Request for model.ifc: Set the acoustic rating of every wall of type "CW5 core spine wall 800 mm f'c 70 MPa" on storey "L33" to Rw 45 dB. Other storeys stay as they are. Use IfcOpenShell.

First a look at what the model holds.

```python
import ifcopenshell
import ifcopenshell.util.element

model = ifcopenshell.open("model.ifc")
print(model.schema)
storey = next(s for s in model.by_type("IfcBuildingStorey") if s.Name == "L33")
walls = [e for e in ifcopenshell.util.element.get_decomposition(storey) if e.is_a("IfcWall")]
seen = {}
for e in walls:
    element_type = ifcopenshell.util.element.get_type(e)
    key = (element_type.Name if element_type != e and element_type else None, ifcopenshell.util.element.get_pset(e, "Pset_WallCommon", "AcousticRating"))
    seen[key] = seen.get(key, 0) + 1
for (name, value), count in sorted(seen.items(), key=str):
    print(count, "x", name, "|", value)
```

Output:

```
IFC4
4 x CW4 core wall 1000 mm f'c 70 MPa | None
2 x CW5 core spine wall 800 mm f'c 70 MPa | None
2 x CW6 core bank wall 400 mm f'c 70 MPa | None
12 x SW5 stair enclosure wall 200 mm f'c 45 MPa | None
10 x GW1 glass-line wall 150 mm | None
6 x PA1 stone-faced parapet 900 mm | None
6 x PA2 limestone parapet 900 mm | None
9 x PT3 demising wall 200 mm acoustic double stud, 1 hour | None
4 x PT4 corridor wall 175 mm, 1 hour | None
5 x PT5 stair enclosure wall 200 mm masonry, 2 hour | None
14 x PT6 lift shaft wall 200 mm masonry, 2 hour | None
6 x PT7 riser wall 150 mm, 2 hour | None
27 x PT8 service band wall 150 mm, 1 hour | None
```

```python
import ifcopenshell
import ifcopenshell.api.pset
import ifcopenshell.util.element

model = ifcopenshell.open("model.ifc")

storey = next(s for s in model.by_type("IfcBuildingStorey") if s.Name == "L33")
walls = [e for e in ifcopenshell.util.element.get_decomposition(storey) if e.is_a("IfcWall")]

count = 0
for e in walls:
    element_type = ifcopenshell.util.element.get_type(e)
    if element_type in (None, e) or element_type.Name != "CW5 core spine wall 800 mm f'c 70 MPa":
        continue
    found = ifcopenshell.util.element.get_pset(e, "Pset_WallCommon", should_inherit=False)
    if found:
        pset = model.by_id(found["id"])
        if len(ifcopenshell.util.element.get_elements_by_pset(pset)) > 1:
            pset = ifcopenshell.api.pset.unshare_pset(model, products=[e], pset=pset)[0]
    else:
        pset = ifcopenshell.api.pset.add_pset(model, product=e, name="Pset_WallCommon")
    ifcopenshell.api.pset.edit_pset(model, pset=pset, properties={"AcousticRating": "Rw 45 dB"})
    count += 1

print(count, "walls updated")

model.write("model_v2.ifc")
```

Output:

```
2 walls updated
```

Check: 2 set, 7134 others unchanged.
